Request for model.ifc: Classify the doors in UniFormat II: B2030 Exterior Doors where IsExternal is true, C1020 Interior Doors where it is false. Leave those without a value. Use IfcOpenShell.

First a look at what the model holds.

```python
import ifcopenshell
import ifcopenshell.util.element

model = ifcopenshell.open("model.ifc")
print(model.schema)
print("classifications:", [c.Name for c in model.by_type("IfcClassification")])
values = [ifcopenshell.util.element.get_pset(e, "Pset_DoorCommon", "IsExternal") for e in model.by_type("IfcDoor")]
for value in (True, False, None):
    print("IsExternal", value, values.count(value))
```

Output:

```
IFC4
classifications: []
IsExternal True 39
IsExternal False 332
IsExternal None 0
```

```python
import ifcopenshell
import ifcopenshell.api.classification
import ifcopenshell.util.element

model = ifcopenshell.open("model.ifc")

system = ifcopenshell.api.classification.add_classification(model, classification="UniFormat II")

doors = model.by_type("IfcDoor")
external = {e: ifcopenshell.util.element.get_pset(e, "Pset_DoorCommon", "IsExternal") for e in doors}
for flag, code, name in ((True, "B2030", "Exterior Doors"), (False, "C1020", "Interior Doors")):
    products = [e for e in doors if external[e] is flag]
    ifcopenshell.api.classification.add_reference(
        model, products=products, classification=system, identification=code, name=name
    )
    print(code, len(products))

model.write("model-out.ifc")
```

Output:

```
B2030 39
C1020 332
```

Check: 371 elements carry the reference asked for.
